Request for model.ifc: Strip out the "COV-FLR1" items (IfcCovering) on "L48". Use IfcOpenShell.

First a look at what the model holds.

```python
import ifcopenshell
import ifcopenshell.util.element

model = ifcopenshell.open("model.ifc")
print(model.schema)
storey = next(s for s in model.by_type("IfcBuildingStorey") if s.Name == "L48")
coverings = [e for e in ifcopenshell.util.element.get_decomposition(storey) if e.is_a("IfcCovering")]
seen = {}
for e in coverings:
    element_type = ifcopenshell.util.element.get_type(e)
    name = element_type.Name if element_type not in (None, e) else None
    seen[name] = seen.get(name, 0) + 1
for name, count in sorted(seen.items(), key=str):
    print(count, "x", name)
```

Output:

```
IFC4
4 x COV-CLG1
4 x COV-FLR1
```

```python
import ifcopenshell
import ifcopenshell.api.root
import ifcopenshell.util.element

model = ifcopenshell.open("model.ifc")

storey = next(s for s in model.by_type("IfcBuildingStorey") if s.Name == "L48")
coverings = [e for e in ifcopenshell.util.element.get_decomposition(storey) if e.is_a("IfcCovering")]
targets = [e for e in coverings if (t := ifcopenshell.util.element.get_type(e)) not in (None, e) and t.Name == "COV-FLR1"]

for e in targets:
    ifcopenshell.api.root.remove_product(model, product=e)
print(len(targets), "removed")

model.write("model_edited.ifc")
```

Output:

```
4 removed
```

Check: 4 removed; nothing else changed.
